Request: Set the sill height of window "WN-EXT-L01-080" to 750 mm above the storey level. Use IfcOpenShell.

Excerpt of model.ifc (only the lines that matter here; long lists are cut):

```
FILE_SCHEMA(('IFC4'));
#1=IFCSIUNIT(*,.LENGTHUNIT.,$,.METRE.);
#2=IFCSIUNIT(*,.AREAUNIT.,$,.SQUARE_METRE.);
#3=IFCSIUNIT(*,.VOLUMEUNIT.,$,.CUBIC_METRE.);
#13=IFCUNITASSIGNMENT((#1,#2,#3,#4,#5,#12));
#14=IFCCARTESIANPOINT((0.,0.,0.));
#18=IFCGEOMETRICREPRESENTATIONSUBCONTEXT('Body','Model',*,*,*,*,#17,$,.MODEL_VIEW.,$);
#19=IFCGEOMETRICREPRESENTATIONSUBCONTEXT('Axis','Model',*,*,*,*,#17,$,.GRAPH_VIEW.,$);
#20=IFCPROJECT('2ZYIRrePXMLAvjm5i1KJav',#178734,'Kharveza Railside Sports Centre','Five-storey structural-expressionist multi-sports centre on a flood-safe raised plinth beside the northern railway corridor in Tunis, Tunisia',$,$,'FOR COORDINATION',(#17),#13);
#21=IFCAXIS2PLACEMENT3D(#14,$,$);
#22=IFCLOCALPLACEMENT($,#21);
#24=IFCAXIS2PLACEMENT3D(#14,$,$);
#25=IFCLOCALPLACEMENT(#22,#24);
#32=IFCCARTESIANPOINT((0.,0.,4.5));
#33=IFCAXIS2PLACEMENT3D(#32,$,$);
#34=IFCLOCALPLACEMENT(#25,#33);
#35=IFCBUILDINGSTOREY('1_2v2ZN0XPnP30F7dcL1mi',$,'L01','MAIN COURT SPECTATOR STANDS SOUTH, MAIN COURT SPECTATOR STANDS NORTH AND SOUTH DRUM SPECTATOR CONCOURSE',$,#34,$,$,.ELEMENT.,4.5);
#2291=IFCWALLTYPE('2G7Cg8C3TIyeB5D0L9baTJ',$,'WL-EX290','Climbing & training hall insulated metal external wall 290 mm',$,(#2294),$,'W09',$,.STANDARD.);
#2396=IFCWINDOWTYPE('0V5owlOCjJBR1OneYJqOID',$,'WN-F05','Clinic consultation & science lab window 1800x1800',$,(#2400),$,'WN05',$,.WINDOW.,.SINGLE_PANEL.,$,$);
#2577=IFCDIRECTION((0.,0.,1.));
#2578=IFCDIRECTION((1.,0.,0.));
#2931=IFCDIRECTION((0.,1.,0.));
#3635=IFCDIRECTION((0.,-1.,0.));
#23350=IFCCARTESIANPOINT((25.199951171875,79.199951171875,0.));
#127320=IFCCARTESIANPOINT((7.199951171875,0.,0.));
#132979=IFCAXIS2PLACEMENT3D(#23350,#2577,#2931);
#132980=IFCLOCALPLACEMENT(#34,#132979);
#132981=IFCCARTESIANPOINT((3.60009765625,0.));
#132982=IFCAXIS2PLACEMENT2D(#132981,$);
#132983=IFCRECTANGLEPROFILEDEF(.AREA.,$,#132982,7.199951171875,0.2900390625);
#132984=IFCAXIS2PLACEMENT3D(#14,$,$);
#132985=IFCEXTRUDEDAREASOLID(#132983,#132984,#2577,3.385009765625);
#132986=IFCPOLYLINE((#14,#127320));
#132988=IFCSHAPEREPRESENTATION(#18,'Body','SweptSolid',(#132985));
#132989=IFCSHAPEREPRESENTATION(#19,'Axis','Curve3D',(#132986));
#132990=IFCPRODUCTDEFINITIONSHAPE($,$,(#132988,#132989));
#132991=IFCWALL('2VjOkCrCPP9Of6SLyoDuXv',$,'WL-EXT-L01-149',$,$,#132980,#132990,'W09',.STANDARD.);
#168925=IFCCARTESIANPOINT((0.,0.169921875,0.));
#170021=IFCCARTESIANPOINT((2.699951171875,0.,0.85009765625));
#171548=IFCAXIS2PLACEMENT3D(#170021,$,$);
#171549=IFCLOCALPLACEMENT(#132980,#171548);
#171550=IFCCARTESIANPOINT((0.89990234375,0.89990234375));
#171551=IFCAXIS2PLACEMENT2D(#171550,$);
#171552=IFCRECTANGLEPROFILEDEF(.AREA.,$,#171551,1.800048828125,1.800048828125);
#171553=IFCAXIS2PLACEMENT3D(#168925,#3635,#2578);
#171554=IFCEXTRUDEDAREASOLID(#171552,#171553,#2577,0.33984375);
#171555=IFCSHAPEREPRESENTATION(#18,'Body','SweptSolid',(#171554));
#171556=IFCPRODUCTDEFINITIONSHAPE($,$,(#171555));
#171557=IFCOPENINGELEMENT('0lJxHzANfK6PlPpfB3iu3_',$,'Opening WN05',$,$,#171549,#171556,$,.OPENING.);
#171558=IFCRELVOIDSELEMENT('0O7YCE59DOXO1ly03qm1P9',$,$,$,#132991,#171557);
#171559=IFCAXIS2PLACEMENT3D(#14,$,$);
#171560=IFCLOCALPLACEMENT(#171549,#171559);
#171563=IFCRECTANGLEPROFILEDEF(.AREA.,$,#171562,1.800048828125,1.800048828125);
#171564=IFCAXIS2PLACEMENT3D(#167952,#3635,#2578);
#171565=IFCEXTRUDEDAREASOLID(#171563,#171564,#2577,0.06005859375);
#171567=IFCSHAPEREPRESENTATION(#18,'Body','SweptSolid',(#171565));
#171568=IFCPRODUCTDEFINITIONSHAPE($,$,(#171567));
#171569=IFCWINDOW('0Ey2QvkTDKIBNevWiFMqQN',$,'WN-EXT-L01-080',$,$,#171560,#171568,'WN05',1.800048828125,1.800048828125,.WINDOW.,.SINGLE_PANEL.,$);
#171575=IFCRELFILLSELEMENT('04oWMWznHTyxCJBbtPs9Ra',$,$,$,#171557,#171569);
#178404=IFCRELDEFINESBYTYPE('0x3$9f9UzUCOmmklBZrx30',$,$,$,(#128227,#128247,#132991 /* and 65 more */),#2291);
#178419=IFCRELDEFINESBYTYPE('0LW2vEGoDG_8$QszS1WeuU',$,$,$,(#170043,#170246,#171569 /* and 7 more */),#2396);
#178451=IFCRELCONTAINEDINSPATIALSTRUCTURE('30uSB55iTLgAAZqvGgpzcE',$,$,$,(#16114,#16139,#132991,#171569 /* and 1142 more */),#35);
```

```python
import numpy as np
import ifcopenshell
import ifcopenshell.api.geometry
import ifcopenshell.geom
import ifcopenshell.util.element
import ifcopenshell.util.placement
import ifcopenshell.util.shape
import ifcopenshell.util.unit

model = ifcopenshell.open("model.ifc")
unit_scale = ifcopenshell.util.unit.calculate_unit_scale(model)

window = model.by_guid("0Ey2QvkTDKIBNevWiFMqQN")
opening = window.FillsVoids[0].RelatingOpeningElement
storey = ifcopenshell.util.element.get_container(window, ifc_class="IfcBuildingStorey")
level = ifcopenshell.util.placement.get_local_placement(storey.ObjectPlacement)[2, 3]

# The opening's origin need not be at the sill, so measure its lowest point.
shape = ifcopenshell.geom.create_shape(ifcopenshell.geom.settings(), opening)
bottom = ifcopenshell.util.shape.get_shape_bottom_elevation(shape, shape.geometry) / unit_scale
dz = level + 0.75 - bottom

shift = np.array([0.0, 0.0, dz])
# The window is placed relative to its opening, so it follows when the opening moves.
matrix = ifcopenshell.util.placement.get_local_placement(opening.ObjectPlacement)
matrix[:3, 3] += shift
ifcopenshell.api.geometry.edit_object_placement(
    model, product=opening, matrix=matrix, is_si=False, should_transform_children=True
)

print(f"moved by {dz * unit_scale:+.3f} m")

model.write("model_edited.ifc")
```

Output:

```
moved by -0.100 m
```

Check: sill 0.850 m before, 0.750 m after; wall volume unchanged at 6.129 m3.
